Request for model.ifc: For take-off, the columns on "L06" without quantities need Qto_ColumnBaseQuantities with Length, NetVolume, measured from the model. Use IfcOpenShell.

First a look at what the model holds.

```python
import ifcopenshell
import ifcopenshell.util.element
import ifcopenshell.util.unit

model = ifcopenshell.open("model.ifc")
print(model.schema)
for unit_type in ("LENGTHUNIT", "AREAUNIT", "VOLUMEUNIT"):
    print(unit_type, ifcopenshell.util.unit.calculate_unit_scale(model, unit_type))
storey = next(s for s in model.by_type("IfcBuildingStorey") if s.Name == "L06")
columns = [e for e in ifcopenshell.util.element.get_decomposition(storey) if e.is_a("IfcColumn")]
for e in sorted(columns, key=lambda e: e.id()):
    print(e.id(), e.is_a(), e.Name, list(ifcopenshell.util.element.get_psets(e, qtos_only=True)), sep=" | ")
```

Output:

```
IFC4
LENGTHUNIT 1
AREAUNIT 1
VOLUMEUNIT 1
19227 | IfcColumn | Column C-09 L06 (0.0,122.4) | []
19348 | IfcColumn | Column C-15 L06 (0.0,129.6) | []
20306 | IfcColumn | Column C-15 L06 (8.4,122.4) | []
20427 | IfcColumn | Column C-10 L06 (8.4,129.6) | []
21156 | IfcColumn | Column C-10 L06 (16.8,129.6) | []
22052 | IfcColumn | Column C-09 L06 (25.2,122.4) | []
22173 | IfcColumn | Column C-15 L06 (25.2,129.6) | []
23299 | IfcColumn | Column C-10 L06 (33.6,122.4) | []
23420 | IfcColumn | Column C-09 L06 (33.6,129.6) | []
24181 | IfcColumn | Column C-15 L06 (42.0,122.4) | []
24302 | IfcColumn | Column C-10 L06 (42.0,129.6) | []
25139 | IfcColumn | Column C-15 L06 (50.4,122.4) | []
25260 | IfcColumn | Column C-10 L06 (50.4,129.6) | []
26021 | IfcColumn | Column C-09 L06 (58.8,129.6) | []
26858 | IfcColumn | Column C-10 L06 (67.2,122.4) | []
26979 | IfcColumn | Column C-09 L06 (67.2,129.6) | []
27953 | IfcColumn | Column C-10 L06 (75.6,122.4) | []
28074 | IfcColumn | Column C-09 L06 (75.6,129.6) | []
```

```python
import ifcopenshell
import ifcopenshell.api.pset
import ifcopenshell.geom
import ifcopenshell.util.element
import ifcopenshell.util.shape
import ifcopenshell.util.unit

model = ifcopenshell.open("model.ifc")
unit_scale = ifcopenshell.util.unit.calculate_unit_scale(model)
volume_scale = ifcopenshell.util.unit.calculate_unit_scale(model, "VOLUMEUNIT")
settings = ifcopenshell.geom.settings()

storey = next(s for s in model.by_type("IfcBuildingStorey") if s.Name == "L06")
columns = [e for e in ifcopenshell.util.element.get_decomposition(storey) if e.is_a("IfcColumn")]

for e in sorted(columns, key=lambda e: e.id()):
    if ifcopenshell.util.element.get_psets(e, qtos_only=True, should_inherit=False):
        continue
    # Geometry comes back in metres, in the element's own axes.
    shape = ifcopenshell.geom.create_shape(settings, e)
    values = {
        "Length": ifcopenshell.util.shape.get_z(shape.geometry) / unit_scale,
        "NetVolume": ifcopenshell.util.shape.get_volume(shape.geometry) / volume_scale,
    }
    qto = ifcopenshell.api.pset.add_qto(model, product=e, name="Qto_ColumnBaseQuantities")
    ifcopenshell.api.pset.edit_qto(model, qto=qto, properties=values)
    print(e.id(), {k: round(v, 3) for k, v in values.items()})

model.write("model_rev.ifc")
```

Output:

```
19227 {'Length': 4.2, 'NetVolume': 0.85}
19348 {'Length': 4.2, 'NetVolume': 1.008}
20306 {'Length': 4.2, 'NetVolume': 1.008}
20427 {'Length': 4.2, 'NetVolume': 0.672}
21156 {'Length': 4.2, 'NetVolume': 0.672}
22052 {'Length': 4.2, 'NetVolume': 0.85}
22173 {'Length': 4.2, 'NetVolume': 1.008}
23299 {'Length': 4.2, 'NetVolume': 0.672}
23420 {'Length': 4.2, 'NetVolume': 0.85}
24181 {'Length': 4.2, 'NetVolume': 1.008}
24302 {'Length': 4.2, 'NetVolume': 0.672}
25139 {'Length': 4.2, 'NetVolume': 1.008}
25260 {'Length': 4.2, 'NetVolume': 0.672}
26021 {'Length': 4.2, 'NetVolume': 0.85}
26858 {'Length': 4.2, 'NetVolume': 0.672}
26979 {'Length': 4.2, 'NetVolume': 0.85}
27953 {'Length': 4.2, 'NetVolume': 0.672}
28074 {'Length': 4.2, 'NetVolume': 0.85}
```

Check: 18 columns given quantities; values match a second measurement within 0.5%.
